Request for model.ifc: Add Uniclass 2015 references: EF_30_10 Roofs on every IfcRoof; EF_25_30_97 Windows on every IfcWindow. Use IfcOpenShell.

First a look at what the model holds.

```python
import ifcopenshell

model = ifcopenshell.open("model.ifc")
print(model.schema)
print("classifications:", [c.Name for c in model.by_type("IfcClassification")])
for ifc_class in ("IfcDoor", "IfcRoof", "IfcStair", "IfcWall", "IfcWindow"):
    print(ifc_class, len(model.by_type(ifc_class)))
```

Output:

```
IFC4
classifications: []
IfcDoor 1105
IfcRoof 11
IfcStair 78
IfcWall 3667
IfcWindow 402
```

```python
import ifcopenshell
import ifcopenshell.api.classification

model = ifcopenshell.open("model.ifc")

system = ifcopenshell.api.classification.add_classification(model, classification="Uniclass 2015")

codes = {
    "IfcRoof": ("EF_30_10", "Roofs"),
    "IfcWindow": ("EF_25_30_97", "Windows"),
}
for ifc_class, (code, name) in codes.items():
    products = model.by_type(ifc_class)
    ifcopenshell.api.classification.add_reference(
        model, products=products, classification=system, identification=code, name=name
    )
    print(code, len(products))

model.write("model_edited.ifc")
```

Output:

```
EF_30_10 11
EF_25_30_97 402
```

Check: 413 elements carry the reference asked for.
